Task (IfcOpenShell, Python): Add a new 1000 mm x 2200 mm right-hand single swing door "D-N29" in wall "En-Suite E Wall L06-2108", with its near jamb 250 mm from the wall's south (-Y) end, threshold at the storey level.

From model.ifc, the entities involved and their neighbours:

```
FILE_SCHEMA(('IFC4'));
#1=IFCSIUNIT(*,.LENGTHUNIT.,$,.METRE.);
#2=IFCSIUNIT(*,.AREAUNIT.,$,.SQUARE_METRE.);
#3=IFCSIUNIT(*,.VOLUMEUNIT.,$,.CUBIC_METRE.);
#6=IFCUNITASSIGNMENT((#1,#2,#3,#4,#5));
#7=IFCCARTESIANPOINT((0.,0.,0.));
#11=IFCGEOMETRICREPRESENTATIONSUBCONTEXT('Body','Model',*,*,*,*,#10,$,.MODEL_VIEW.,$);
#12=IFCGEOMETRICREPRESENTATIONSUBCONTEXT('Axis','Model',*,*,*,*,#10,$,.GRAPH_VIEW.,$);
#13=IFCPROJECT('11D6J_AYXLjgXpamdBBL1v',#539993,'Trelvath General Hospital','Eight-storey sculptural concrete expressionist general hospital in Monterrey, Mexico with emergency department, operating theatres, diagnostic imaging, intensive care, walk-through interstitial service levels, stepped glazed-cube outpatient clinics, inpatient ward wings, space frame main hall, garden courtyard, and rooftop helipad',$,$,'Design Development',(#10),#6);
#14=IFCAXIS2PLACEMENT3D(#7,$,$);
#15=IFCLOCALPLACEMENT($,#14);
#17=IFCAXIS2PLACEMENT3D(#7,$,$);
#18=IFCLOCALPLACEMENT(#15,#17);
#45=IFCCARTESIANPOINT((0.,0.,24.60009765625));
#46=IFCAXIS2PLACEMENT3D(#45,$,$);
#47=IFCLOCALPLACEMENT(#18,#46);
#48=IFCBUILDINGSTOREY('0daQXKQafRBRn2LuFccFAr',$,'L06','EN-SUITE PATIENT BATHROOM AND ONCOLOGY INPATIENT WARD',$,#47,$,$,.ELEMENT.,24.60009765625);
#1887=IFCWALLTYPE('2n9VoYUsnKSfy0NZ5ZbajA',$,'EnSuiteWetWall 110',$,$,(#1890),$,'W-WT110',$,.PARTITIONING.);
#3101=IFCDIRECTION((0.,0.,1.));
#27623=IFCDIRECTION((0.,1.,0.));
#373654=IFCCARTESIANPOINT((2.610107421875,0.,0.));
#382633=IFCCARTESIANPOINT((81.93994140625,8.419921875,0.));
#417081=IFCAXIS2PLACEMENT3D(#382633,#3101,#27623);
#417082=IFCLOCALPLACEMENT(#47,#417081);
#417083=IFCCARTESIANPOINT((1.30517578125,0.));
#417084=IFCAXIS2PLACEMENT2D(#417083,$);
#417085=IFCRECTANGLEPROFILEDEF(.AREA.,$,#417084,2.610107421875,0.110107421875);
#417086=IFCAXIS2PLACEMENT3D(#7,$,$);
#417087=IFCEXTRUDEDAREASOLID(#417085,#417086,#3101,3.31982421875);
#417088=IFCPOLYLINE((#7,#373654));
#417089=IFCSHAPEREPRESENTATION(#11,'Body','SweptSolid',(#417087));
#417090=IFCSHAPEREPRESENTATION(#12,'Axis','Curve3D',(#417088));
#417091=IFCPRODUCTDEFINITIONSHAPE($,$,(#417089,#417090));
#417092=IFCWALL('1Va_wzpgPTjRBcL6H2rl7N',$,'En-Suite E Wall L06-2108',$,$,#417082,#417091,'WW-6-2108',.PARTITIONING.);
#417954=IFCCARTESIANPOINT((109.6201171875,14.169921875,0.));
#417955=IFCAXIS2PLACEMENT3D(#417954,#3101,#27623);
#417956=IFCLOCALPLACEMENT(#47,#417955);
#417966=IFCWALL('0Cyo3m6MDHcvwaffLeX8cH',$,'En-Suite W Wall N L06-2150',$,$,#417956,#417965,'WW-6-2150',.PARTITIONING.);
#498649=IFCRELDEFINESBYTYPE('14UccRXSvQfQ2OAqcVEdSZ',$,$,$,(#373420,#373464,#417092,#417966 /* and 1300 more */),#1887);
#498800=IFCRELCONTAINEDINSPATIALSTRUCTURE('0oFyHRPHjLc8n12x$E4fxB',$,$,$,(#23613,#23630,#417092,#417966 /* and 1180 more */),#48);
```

```python
import numpy as np
import ifcopenshell
import ifcopenshell.api.feature
import ifcopenshell.api.geometry
import ifcopenshell.api.root
import ifcopenshell.api.spatial
import ifcopenshell.geom
import ifcopenshell.util.element
import ifcopenshell.util.placement
import ifcopenshell.util.representation
import ifcopenshell.util.shape
import ifcopenshell.util.unit

model = ifcopenshell.open("model.ifc")
unit_scale = ifcopenshell.util.unit.calculate_unit_scale(model)
settings = ifcopenshell.geom.settings()


def volume(element):
    """Net volume in cubic metres, openings subtracted."""
    shape = ifcopenshell.geom.create_shape(settings, element)
    return ifcopenshell.util.shape.get_volume(shape.geometry)


wall = model.by_guid("1Va_wzpgPTjRBcL6H2rl7N")
storey = ifcopenshell.util.element.get_container(wall, ifc_class="IfcBuildingStorey")
context = ifcopenshell.util.representation.get_context(model, "Model", "Body", "MODEL_VIEW")
before = volume(wall)

width, height, from_end, sill = 1, 2.2, 0.25, 0.0  # metres

# The wall runs along its own X axis, and the end named is its -X end.
wall_shape = ifcopenshell.geom.create_shape(settings, wall)
x, y, z = ifcopenshell.util.shape.get_vertices(wall_shape.geometry).T
start = x.min() + from_end
face, thickness = float(y.min()), float(y.max() - y.min())
wall_matrix = ifcopenshell.util.placement.get_local_placement(wall.ObjectPlacement)
level = ifcopenshell.util.placement.get_local_placement(storey.ObjectPlacement)[2, 3]


def in_wall(x, y):
    """Placement at x, y metres in the wall's axes, at sill height."""
    matrix = wall_matrix.copy()
    matrix[:, 3] = wall_matrix @ np.array([x / unit_scale, y / unit_scale, 0.0, 1.0])
    matrix[2, 3] = level + sill / unit_scale
    return matrix


# Opening: a box that overshoots both wall faces by 50 mm.
opening = ifcopenshell.api.root.create_entity(model, ifc_class="IfcOpeningElement", predefined_type="OPENING")
box = ifcopenshell.api.geometry.add_wall_representation(
    model, context=context, length=width, height=height, thickness=thickness + 0.1
)
ifcopenshell.api.geometry.assign_representation(model, product=opening, representation=box)
ifcopenshell.api.geometry.edit_object_placement(model, product=opening, matrix=in_wall(start, face - 0.05), is_si=False)
ifcopenshell.api.feature.add_feature(model, feature=opening, element=wall)

door = ifcopenshell.api.root.create_entity(model, ifc_class="IfcDoor", name="D-N29", predefined_type="DOOR")
door.OverallWidth, door.OverallHeight = width / unit_scale, height / unit_scale
door.OperationType = "SINGLE_SWING_RIGHT"
body = ifcopenshell.api.geometry.add_door_representation(
    model,
    context=context,
    overall_width=door.OverallWidth,
    overall_height=door.OverallHeight,
    operation_type="SINGLE_SWING_RIGHT",
    lining_properties={"LiningDepth": thickness / unit_scale, "ThresholdDepth": thickness / unit_scale},
)
ifcopenshell.api.geometry.assign_representation(model, product=door, representation=body)
ifcopenshell.api.spatial.assign_container(model, products=[door], relating_structure=storey)
ifcopenshell.api.feature.add_filling(model, opening=opening, element=door)

# The lining spans the wall, so the door starts at the wall face.
ifcopenshell.api.geometry.edit_object_placement(model, product=door, matrix=in_wall(start, face), is_si=False)

after = volume(wall)

print(f"wall volume {before:.3f} -> {after:.3f} m3")

model.write("model-out.ifc")
```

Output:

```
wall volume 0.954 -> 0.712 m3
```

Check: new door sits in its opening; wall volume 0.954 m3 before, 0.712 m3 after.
